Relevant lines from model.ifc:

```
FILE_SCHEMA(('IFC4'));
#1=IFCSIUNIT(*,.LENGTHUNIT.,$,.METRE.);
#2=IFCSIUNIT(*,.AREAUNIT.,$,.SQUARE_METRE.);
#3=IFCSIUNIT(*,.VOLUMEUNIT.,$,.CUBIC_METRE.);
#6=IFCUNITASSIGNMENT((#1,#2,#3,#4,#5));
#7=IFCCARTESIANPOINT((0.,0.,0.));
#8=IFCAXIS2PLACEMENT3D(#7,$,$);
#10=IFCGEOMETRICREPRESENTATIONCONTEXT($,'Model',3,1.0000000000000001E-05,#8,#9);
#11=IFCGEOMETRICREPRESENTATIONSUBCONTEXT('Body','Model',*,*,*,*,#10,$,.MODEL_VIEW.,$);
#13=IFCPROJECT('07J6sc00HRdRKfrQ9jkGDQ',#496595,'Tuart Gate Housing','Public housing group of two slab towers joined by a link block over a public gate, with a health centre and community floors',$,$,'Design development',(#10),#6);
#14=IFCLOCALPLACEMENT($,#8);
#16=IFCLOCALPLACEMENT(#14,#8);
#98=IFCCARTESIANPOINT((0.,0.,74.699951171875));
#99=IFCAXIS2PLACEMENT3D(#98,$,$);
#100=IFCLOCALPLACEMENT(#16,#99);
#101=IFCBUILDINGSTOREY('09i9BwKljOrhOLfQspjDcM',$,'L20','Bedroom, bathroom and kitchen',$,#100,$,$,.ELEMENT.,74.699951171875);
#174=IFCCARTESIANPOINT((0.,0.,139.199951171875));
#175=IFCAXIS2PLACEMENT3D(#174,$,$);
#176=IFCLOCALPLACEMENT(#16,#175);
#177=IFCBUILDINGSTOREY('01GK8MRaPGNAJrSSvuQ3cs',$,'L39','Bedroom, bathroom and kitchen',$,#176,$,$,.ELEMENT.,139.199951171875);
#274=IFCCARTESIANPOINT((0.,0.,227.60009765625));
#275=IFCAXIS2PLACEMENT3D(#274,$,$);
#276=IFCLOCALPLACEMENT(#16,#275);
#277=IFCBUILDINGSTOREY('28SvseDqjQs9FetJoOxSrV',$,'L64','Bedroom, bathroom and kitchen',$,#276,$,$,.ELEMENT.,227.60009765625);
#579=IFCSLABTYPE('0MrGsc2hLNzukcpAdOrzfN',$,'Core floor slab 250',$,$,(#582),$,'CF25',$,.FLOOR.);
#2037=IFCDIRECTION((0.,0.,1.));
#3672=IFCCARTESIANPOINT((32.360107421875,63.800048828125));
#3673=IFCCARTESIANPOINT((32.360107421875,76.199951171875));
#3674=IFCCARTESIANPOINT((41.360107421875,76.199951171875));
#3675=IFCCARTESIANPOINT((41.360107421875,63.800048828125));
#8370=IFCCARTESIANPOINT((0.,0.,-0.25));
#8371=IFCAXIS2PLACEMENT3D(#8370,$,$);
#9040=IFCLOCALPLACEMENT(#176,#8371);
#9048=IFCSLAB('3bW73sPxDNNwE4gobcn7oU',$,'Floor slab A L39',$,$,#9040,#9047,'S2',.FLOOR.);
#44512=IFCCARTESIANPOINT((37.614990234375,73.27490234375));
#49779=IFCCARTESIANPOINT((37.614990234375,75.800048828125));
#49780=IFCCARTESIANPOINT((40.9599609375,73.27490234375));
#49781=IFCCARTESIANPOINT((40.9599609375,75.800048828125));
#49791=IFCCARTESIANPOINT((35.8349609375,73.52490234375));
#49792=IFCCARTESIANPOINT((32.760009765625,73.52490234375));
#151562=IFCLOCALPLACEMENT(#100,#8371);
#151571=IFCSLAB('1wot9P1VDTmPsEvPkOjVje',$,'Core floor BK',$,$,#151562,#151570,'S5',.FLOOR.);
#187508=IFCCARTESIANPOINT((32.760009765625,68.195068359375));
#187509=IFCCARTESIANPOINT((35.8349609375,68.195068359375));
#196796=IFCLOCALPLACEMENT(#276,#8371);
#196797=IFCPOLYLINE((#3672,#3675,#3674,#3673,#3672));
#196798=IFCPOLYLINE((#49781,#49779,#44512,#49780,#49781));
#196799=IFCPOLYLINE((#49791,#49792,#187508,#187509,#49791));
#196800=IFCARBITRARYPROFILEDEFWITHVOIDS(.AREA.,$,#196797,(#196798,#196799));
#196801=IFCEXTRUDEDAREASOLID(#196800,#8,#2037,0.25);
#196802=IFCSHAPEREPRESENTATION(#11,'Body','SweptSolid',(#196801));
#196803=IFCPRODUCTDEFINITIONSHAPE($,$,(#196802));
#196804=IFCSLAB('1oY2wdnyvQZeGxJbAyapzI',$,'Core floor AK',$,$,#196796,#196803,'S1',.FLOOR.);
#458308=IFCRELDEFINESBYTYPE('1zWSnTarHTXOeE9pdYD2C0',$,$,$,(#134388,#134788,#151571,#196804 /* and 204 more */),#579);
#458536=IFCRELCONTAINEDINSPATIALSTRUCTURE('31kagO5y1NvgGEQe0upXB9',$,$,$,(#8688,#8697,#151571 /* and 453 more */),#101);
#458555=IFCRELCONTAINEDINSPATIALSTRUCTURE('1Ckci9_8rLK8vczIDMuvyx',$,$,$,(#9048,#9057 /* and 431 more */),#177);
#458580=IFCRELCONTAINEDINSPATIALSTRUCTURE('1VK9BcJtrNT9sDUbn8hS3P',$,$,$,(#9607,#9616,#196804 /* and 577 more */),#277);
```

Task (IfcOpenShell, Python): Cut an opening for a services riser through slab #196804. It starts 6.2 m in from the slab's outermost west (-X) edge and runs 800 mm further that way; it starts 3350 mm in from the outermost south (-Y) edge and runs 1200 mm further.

```python
import numpy as np
import ifcopenshell
import ifcopenshell.api.feature
import ifcopenshell.api.geometry
import ifcopenshell.api.root
import ifcopenshell.geom
import ifcopenshell.util.placement
import ifcopenshell.util.representation
import ifcopenshell.util.shape
import ifcopenshell.util.unit

model = ifcopenshell.open("model.ifc")
unit_scale = ifcopenshell.util.unit.calculate_unit_scale(model)
settings = ifcopenshell.geom.settings()


def volume(element):
    """Net volume in cubic metres, openings subtracted."""
    shape = ifcopenshell.geom.create_shape(settings, element)
    return ifcopenshell.util.shape.get_volume(shape.geometry)


slab = model.by_id(196804)
before = volume(slab)

# Extent in the slab's own axes, in metres. The edges named are its -X and -Y sides.
slab_shape = ifcopenshell.geom.create_shape(settings, slab)
vertices = ifcopenshell.util.shape.get_vertices(slab_shape.geometry)
x_min, y_min, bottom = vertices.min(axis=0)
top = vertices[:, 2].max()

opening = ifcopenshell.api.root.create_entity(model, ifc_class="IfcOpeningElement", name="Services riser opening", predefined_type="OPENING")
context = ifcopenshell.util.representation.get_context(model, "Model", "Body", "MODEL_VIEW")
width, depth = 0.8, 1.2
outline = [(0.0, 0.0), (width, 0.0), (width, depth), (0.0, depth), (0.0, 0.0)]
# Overshoot both faces by 50 mm so the cut is clean.
shape = ifcopenshell.api.geometry.add_slab_representation(
    model, context=context, depth=top - bottom + 0.1, polyline=outline
)
ifcopenshell.api.geometry.assign_representation(model, product=opening, representation=shape)

matrix = ifcopenshell.util.placement.get_local_placement(slab.ObjectPlacement)
matrix[:, 3] = matrix @ np.append(np.array([x_min + 6.2, y_min + 3.35, bottom - 0.05]) / unit_scale, 1.0)
ifcopenshell.api.geometry.edit_object_placement(model, product=opening, matrix=matrix, is_si=False)
ifcopenshell.api.feature.add_feature(model, feature=opening, element=slab)

after = volume(slab)

print(f"slab volume {before:.3f} -> {after:.3f} m3")

model.write("model_rev.ifc")
```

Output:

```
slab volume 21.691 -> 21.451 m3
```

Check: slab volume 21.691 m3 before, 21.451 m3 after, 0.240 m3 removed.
